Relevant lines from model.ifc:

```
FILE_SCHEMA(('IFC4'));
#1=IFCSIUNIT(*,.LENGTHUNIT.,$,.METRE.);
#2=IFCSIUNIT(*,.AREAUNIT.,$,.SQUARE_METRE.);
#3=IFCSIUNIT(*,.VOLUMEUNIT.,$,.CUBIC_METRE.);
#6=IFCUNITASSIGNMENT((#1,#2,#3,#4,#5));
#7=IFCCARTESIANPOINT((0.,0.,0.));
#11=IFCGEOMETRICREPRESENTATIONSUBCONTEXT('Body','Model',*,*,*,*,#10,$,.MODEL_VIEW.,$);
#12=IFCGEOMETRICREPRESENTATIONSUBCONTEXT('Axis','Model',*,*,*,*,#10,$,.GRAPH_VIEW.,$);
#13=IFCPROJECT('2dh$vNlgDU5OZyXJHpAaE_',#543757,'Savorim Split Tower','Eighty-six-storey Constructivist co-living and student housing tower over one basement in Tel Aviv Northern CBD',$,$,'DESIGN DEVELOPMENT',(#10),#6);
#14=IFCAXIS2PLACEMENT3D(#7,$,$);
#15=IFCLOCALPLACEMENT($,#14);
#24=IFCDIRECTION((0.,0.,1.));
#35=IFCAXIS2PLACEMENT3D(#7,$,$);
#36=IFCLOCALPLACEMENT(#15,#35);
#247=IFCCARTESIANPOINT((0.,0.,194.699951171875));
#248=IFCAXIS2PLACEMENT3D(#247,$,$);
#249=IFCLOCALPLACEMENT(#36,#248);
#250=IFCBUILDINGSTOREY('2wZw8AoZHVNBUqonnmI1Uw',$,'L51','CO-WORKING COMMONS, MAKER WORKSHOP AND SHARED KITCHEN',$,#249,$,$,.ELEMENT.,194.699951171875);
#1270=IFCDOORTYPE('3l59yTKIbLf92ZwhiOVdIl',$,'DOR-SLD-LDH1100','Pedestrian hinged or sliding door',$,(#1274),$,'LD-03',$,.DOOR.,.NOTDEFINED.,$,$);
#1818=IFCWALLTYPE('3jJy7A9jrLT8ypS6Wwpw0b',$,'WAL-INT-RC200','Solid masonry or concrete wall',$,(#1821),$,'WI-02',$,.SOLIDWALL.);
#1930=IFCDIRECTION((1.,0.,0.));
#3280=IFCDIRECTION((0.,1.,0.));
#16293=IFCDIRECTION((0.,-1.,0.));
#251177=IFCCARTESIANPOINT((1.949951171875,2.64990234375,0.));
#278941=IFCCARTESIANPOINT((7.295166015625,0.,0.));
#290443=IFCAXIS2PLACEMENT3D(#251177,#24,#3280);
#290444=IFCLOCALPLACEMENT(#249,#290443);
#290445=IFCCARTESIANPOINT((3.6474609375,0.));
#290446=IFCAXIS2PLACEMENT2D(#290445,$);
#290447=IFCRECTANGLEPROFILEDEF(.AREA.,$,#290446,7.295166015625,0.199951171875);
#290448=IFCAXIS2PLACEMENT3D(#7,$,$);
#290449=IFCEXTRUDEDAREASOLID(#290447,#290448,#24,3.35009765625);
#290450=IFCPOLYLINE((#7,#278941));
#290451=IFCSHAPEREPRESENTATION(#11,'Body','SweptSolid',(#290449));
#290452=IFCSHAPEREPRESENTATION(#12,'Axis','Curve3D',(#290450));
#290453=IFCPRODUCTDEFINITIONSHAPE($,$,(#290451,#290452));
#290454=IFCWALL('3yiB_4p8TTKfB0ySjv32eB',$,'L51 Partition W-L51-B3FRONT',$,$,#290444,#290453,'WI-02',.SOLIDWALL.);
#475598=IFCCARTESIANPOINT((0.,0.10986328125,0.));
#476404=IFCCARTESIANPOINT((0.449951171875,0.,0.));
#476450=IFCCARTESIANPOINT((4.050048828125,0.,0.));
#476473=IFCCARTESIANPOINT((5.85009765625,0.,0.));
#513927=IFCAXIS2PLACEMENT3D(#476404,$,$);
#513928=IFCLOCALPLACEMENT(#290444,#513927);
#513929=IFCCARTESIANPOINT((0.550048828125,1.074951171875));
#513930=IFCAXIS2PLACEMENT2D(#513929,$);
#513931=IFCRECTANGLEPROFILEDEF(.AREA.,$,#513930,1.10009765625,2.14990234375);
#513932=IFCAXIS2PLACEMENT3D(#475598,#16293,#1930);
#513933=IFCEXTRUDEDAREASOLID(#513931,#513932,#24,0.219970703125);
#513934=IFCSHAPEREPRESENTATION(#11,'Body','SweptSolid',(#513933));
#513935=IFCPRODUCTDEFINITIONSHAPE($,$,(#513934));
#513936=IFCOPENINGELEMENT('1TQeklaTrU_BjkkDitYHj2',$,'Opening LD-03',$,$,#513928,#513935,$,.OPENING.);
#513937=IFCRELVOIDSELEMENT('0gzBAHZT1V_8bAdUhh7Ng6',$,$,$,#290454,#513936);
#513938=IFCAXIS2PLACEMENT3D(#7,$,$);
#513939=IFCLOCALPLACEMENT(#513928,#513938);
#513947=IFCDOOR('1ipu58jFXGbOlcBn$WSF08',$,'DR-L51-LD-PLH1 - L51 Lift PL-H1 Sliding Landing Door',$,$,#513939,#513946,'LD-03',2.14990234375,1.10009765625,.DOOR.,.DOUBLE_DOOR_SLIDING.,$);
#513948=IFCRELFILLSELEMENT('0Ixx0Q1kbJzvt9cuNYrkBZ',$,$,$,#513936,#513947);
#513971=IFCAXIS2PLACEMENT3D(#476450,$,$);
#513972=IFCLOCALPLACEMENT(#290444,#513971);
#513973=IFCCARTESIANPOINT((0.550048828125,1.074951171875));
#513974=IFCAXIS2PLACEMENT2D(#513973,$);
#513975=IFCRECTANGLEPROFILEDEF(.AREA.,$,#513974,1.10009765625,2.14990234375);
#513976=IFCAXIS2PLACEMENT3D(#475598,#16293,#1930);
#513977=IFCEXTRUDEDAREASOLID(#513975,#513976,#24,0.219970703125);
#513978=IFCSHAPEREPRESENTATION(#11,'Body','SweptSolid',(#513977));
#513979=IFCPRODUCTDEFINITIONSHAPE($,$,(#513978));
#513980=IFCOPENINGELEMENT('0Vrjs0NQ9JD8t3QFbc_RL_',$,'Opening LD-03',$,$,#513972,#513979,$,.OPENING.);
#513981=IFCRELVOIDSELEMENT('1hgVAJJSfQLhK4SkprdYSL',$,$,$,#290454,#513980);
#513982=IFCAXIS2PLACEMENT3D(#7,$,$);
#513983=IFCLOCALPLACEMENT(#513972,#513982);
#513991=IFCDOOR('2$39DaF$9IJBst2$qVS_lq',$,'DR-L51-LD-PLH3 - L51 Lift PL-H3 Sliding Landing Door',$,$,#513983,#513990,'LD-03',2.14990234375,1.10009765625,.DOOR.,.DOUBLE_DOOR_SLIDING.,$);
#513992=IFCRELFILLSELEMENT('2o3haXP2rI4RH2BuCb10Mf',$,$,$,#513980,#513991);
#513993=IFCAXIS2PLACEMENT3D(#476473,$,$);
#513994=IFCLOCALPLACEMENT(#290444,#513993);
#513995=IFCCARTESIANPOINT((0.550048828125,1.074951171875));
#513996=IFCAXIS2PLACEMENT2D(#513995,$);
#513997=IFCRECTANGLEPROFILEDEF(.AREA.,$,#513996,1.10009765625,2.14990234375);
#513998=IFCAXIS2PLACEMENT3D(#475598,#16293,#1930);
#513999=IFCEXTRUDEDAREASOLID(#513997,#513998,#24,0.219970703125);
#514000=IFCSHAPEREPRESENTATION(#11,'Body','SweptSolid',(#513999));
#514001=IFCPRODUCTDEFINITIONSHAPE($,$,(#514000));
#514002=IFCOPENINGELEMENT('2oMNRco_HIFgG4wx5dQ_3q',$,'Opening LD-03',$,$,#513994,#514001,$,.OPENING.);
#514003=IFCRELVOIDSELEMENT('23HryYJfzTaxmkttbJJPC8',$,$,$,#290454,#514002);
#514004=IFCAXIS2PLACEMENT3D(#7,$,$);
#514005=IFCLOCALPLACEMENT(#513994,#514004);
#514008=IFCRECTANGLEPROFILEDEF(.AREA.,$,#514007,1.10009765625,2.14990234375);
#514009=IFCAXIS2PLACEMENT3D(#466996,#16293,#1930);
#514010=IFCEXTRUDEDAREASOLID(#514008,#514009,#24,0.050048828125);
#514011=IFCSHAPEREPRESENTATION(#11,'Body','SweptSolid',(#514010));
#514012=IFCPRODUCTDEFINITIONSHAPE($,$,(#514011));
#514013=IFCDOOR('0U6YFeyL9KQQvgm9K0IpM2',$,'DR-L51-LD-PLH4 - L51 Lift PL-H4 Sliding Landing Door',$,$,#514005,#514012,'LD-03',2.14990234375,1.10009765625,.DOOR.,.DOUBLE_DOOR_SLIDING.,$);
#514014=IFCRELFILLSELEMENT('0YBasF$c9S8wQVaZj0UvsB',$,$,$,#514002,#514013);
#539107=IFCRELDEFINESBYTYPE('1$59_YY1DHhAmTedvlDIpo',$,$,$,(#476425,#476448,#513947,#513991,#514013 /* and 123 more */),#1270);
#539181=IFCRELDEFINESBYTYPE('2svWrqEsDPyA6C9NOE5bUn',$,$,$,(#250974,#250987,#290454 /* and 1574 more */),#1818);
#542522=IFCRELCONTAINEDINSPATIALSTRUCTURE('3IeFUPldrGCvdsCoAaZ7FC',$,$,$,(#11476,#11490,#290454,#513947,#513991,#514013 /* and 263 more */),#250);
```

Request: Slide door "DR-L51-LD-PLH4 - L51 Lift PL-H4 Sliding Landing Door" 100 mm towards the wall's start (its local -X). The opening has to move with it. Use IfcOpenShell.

```python
import ifcopenshell
import ifcopenshell.api.geometry
import ifcopenshell.util.placement

model = ifcopenshell.open("model.ifc")

door = model.by_guid("0U6YFeyL9KQQvgm9K0IpM2")
opening = door.FillsVoids[0].RelatingOpeningElement
wall = opening.VoidsElements[0].RelatingBuildingElement

wall_matrix = ifcopenshell.util.placement.get_local_placement(wall.ObjectPlacement)
shift = wall_matrix[:3, 0] * -0.1
before = ifcopenshell.util.placement.get_local_placement(door.ObjectPlacement)[:3, 3].copy()

# The door is placed relative to its opening, so it follows when the opening moves.
matrix = ifcopenshell.util.placement.get_local_placement(opening.ObjectPlacement)
matrix[:3, 3] += shift
ifcopenshell.api.geometry.edit_object_placement(
    model, product=opening, matrix=matrix, is_si=False, should_transform_children=True
)

after = ifcopenshell.util.placement.get_local_placement(door.ObjectPlacement)[:3, 3]
print("door moved by", (after - before).round(3) + 0.0)

model.write("model_v2.ifc")
```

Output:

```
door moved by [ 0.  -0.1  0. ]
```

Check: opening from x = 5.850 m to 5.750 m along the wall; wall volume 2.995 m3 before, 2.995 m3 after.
